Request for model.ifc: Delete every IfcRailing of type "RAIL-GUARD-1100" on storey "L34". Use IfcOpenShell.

First a look at what the model holds.

```python
import ifcopenshell
import ifcopenshell.util.element

model = ifcopenshell.open("model.ifc")
print(model.schema)
storey = next(s for s in model.by_type("IfcBuildingStorey") if s.Name == "L34")
railings = [e for e in ifcopenshell.util.element.get_decomposition(storey) if e.is_a("IfcRailing")]
seen = {}
for e in railings:
    element_type = ifcopenshell.util.element.get_type(e)
    name = element_type.Name if element_type not in (None, e) else None
    seen[name] = seen.get(name, 0) + 1
for name, count in sorted(seen.items(), key=str):
    print(count, "x", name)
```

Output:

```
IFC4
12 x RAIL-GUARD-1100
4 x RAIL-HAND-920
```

```python
import ifcopenshell
import ifcopenshell.api.root
import ifcopenshell.util.element

model = ifcopenshell.open("model.ifc")

storey = next(s for s in model.by_type("IfcBuildingStorey") if s.Name == "L34")
railings = [e for e in ifcopenshell.util.element.get_decomposition(storey) if e.is_a("IfcRailing")]
targets = [e for e in railings if (t := ifcopenshell.util.element.get_type(e)) not in (None, e) and t.Name == "RAIL-GUARD-1100"]

for e in targets:
    ifcopenshell.api.root.remove_product(model, product=e)
print(len(targets), "removed")

model.write("model_edited.ifc")
```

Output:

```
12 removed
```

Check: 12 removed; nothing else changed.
